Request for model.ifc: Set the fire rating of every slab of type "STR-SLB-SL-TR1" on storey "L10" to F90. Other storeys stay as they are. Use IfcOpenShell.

First a look at what the model holds.

```python
import ifcopenshell
import ifcopenshell.util.element

model = ifcopenshell.open("model.ifc")
print(model.schema)
storey = next(s for s in model.by_type("IfcBuildingStorey") if s.Name == "L10")
slabs = [e for e in ifcopenshell.util.element.get_decomposition(storey) if e.is_a("IfcSlab")]
seen = {}
for e in slabs:
    element_type = ifcopenshell.util.element.get_type(e)
    key = (element_type.Name if element_type != e and element_type else None, ifcopenshell.util.element.get_pset(e, "Pset_SlabCommon", "FireRating"))
    seen[key] = seen.get(key, 0) + 1
for (name, value), count in sorted(seen.items(), key=str):
    print(count, "x", name, "|", value)
```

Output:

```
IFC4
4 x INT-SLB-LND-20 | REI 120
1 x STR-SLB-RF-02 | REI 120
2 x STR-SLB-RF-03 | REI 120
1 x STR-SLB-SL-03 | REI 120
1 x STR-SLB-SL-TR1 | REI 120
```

```python
import ifcopenshell
import ifcopenshell.api.pset
import ifcopenshell.util.element

model = ifcopenshell.open("model.ifc")

storey = next(s for s in model.by_type("IfcBuildingStorey") if s.Name == "L10")
slabs = [e for e in ifcopenshell.util.element.get_decomposition(storey) if e.is_a("IfcSlab")]

count = 0
for e in slabs:
    element_type = ifcopenshell.util.element.get_type(e)
    if element_type in (None, e) or element_type.Name != "STR-SLB-SL-TR1":
        continue
    # add_pset returns the element's existing set when there is one.
    pset = ifcopenshell.api.pset.add_pset(model, product=e, name="Pset_SlabCommon")
    ifcopenshell.api.pset.edit_pset(model, pset=pset, properties={"FireRating": "F90"})
    count += 1

print(count, "slabs updated")

model.write("model_edited.ifc")
```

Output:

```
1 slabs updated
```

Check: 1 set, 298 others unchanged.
